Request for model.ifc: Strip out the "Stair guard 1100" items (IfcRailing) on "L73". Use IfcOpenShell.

First a look at what the model holds.

```python
import ifcopenshell
import ifcopenshell.util.element

model = ifcopenshell.open("model.ifc")
print(model.schema)
storey = next(s for s in model.by_type("IfcBuildingStorey") if s.Name == "L73")
railings = [e for e in ifcopenshell.util.element.get_decomposition(storey) if e.is_a("IfcRailing")]
seen = {}
for e in railings:
    element_type = ifcopenshell.util.element.get_type(e)
    name = element_type.Name if element_type not in (None, e) else None
    seen[name] = seen.get(name, 0) + 1
for name, count in sorted(seen.items(), key=str):
    print(count, "x", name)
```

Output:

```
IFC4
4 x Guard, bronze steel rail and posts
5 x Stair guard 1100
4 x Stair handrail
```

```python
import ifcopenshell
import ifcopenshell.api.root
import ifcopenshell.util.element

model = ifcopenshell.open("model.ifc")

storey = next(s for s in model.by_type("IfcBuildingStorey") if s.Name == "L73")
railings = [e for e in ifcopenshell.util.element.get_decomposition(storey) if e.is_a("IfcRailing")]
targets = [e for e in railings if (t := ifcopenshell.util.element.get_type(e)) not in (None, e) and t.Name == "Stair guard 1100"]

for e in targets:
    ifcopenshell.api.root.remove_product(model, product=e)
print(len(targets), "removed")

model.write("model_v2.ifc")
```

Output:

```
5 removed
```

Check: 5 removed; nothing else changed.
